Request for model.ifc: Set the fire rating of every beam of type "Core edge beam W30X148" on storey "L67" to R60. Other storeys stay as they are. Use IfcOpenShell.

First a look at what the model holds.

```python
import ifcopenshell
import ifcopenshell.util.element

model = ifcopenshell.open("model.ifc")
print(model.schema)
storey = next(s for s in model.by_type("IfcBuildingStorey") if s.Name == "L67")
beams = [e for e in ifcopenshell.util.element.get_decomposition(storey) if e.is_a("IfcBeam")]
seen = {}
for e in beams:
    element_type = ifcopenshell.util.element.get_type(e)
    key = (element_type.Name if element_type != e and element_type else None, ifcopenshell.util.element.get_pset(e, "Pset_BeamCommon", "FireRating"))
    seen[key] = seen.get(key, 0) + 1
for (name, value), count in sorted(seen.items(), key=str):
    print(count, "x", name, "|", value)
```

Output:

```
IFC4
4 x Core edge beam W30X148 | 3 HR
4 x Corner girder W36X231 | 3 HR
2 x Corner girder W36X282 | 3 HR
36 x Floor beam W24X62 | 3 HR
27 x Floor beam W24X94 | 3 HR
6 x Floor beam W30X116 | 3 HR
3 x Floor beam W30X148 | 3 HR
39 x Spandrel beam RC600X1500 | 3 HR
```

```python
import ifcopenshell
import ifcopenshell.api.pset
import ifcopenshell.util.element

model = ifcopenshell.open("model.ifc")

storey = next(s for s in model.by_type("IfcBuildingStorey") if s.Name == "L67")
beams = [e for e in ifcopenshell.util.element.get_decomposition(storey) if e.is_a("IfcBeam")]

count = 0
for e in beams:
    element_type = ifcopenshell.util.element.get_type(e)
    if element_type in (None, e) or element_type.Name != "Core edge beam W30X148":
        continue
    found = ifcopenshell.util.element.get_pset(e, "Pset_BeamCommon", should_inherit=False)
    if found:
        pset = model.by_id(found["id"])
        if len(ifcopenshell.util.element.get_elements_by_pset(pset)) > 1:
            pset = ifcopenshell.api.pset.unshare_pset(model, products=[e], pset=pset)[0]
    else:
        pset = ifcopenshell.api.pset.add_pset(model, product=e, name="Pset_BeamCommon")
    ifcopenshell.api.pset.edit_pset(model, pset=pset, properties={"FireRating": "R60"})
    count += 1

print(count, "beams updated")

model.write("model_rev.ifc")
```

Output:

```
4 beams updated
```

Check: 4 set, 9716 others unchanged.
